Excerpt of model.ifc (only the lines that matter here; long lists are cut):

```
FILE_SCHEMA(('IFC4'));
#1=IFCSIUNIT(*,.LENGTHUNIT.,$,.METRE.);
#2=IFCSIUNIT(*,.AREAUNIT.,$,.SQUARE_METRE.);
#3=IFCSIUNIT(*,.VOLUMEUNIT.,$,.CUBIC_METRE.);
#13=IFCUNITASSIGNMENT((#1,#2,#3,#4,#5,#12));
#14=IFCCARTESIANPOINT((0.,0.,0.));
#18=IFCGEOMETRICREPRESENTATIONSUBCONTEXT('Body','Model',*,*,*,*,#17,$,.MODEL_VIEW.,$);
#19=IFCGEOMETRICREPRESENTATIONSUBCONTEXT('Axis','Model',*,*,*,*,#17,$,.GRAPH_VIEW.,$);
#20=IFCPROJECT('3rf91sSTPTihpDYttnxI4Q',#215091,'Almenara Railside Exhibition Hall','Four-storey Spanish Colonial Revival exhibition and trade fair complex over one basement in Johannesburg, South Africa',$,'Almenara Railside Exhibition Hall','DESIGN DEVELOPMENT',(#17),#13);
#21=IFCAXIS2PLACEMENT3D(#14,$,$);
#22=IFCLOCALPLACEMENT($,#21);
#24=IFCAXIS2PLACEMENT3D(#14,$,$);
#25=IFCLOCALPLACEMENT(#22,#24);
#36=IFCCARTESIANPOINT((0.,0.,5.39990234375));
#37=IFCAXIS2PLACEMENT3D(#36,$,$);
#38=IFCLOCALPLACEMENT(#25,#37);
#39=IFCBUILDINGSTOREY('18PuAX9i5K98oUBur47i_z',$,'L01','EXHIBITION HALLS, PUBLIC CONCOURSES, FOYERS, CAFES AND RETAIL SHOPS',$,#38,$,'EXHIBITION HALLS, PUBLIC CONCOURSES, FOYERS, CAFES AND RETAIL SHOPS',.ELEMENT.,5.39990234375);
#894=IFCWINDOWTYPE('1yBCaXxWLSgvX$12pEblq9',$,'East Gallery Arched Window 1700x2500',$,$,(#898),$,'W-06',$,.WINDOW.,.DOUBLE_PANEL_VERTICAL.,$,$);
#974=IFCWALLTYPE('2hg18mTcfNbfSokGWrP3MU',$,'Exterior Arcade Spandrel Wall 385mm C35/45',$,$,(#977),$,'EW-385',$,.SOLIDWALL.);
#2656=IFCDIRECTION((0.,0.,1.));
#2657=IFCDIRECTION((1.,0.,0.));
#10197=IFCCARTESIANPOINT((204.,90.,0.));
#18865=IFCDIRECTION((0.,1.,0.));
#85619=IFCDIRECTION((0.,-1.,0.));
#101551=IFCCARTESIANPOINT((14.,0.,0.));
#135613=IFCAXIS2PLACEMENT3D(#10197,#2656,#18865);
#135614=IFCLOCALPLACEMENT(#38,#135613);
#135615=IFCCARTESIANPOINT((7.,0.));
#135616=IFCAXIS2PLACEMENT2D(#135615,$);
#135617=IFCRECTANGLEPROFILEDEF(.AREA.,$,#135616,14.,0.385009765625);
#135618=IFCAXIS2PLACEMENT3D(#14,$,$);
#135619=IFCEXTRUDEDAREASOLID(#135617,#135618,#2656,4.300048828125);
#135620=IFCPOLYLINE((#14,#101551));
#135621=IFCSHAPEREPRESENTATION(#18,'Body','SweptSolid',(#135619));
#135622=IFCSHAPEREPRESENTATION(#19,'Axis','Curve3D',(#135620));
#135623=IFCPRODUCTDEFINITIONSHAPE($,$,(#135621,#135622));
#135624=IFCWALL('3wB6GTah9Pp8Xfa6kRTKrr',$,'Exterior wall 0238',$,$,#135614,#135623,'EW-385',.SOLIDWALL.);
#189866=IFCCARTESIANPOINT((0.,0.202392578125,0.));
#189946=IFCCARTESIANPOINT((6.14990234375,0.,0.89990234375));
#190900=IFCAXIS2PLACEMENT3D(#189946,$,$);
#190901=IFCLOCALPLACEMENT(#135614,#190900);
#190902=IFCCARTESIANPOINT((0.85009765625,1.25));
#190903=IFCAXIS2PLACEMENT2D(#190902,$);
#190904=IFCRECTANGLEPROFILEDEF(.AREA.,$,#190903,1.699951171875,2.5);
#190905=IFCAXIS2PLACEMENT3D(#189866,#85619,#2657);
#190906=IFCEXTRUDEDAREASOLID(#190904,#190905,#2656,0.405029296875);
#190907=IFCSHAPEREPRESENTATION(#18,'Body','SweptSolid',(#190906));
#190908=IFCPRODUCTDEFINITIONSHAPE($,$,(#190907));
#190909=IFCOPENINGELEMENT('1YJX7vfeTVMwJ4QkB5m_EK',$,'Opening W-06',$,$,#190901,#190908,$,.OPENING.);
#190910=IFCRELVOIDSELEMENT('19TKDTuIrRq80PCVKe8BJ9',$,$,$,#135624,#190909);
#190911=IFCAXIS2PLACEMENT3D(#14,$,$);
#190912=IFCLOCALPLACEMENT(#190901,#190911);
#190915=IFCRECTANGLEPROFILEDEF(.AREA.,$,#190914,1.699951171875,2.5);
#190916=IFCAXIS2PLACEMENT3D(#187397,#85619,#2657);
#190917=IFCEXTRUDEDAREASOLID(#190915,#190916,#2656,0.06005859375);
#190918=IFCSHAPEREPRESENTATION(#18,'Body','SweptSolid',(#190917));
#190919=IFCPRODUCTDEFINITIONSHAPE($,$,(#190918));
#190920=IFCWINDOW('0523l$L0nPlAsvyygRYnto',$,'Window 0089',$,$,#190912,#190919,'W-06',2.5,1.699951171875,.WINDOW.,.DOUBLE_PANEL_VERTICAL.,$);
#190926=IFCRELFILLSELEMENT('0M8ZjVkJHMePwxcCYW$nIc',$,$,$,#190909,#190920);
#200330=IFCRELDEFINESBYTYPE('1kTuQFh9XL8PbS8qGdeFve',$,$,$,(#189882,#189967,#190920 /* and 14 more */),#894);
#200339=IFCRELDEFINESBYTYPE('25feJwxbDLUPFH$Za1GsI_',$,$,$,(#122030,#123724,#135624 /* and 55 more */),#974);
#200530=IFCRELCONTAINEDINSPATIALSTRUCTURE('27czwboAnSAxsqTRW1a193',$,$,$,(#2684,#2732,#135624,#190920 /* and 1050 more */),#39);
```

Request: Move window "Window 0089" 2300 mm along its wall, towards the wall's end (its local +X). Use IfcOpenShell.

```python
import ifcopenshell
import ifcopenshell.api.geometry
import ifcopenshell.util.placement

model = ifcopenshell.open("model.ifc")

window = model.by_id(190920)
opening = window.FillsVoids[0].RelatingOpeningElement
wall = opening.VoidsElements[0].RelatingBuildingElement

wall_matrix = ifcopenshell.util.placement.get_local_placement(wall.ObjectPlacement)
shift = wall_matrix[:3, 0] * 2.3
before = ifcopenshell.util.placement.get_local_placement(window.ObjectPlacement)[:3, 3].copy()

# The window is placed relative to its opening, so it follows when the opening moves.
matrix = ifcopenshell.util.placement.get_local_placement(opening.ObjectPlacement)
matrix[:3, 3] += shift
ifcopenshell.api.geometry.edit_object_placement(
    model, product=opening, matrix=matrix, is_si=False, should_transform_children=True
)

after = ifcopenshell.util.placement.get_local_placement(window.ObjectPlacement)[:3, 3]
print("window moved by", (after - before).round(3) + 0.0)

model.write("model_updated.ifc")
```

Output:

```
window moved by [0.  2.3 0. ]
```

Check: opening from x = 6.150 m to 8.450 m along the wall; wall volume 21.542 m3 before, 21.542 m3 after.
